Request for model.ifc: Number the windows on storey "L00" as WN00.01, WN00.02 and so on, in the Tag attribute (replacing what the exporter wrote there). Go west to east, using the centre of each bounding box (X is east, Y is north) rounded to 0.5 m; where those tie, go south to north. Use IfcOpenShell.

First a look at what the model holds.

```python
import ifcopenshell
import ifcopenshell.util.element
import ifcopenshell.util.placement

model = ifcopenshell.open("model.ifc")
print(model.schema)
storey = next(s for s in model.by_type("IfcBuildingStorey") if s.Name == "L00")
windows = [e for e in ifcopenshell.util.element.get_decomposition(storey) if e.is_a("IfcWindow")]
for e in sorted(windows, key=lambda e: e.id()):
    origin = ifcopenshell.util.placement.get_local_placement(e.ObjectPlacement)[:3, 3]
    print(e.id(), e.Tag, e.Name, origin.round(2) + 0.0, sep=" | ")
```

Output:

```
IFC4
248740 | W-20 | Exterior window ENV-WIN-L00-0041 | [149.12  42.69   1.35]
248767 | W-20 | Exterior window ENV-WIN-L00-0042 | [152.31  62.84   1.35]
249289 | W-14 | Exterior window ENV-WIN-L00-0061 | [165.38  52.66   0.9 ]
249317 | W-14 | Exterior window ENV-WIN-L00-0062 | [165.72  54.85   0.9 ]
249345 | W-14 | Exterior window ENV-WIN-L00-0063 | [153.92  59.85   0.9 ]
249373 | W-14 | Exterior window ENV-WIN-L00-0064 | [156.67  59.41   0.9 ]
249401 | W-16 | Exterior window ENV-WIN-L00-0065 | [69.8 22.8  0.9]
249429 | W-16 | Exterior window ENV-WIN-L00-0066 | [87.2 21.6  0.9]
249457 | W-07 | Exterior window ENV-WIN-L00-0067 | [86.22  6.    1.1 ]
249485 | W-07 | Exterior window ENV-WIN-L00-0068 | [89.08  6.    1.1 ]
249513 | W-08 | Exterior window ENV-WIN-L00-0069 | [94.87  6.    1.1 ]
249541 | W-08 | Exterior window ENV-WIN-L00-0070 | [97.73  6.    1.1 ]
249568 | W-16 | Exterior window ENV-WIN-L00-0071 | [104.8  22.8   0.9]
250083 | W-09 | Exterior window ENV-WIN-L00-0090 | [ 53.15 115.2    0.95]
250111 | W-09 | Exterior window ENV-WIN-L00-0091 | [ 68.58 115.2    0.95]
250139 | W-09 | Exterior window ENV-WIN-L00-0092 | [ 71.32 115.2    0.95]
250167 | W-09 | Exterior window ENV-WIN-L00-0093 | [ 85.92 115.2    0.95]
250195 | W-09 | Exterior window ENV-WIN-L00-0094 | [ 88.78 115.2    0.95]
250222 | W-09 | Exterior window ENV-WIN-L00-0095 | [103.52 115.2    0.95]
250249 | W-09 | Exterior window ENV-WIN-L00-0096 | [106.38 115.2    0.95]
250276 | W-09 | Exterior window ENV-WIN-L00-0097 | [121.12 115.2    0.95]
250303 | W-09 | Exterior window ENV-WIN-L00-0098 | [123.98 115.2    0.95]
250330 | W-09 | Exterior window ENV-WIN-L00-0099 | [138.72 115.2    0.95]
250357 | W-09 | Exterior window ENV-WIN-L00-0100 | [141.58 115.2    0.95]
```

```python
import ifcopenshell
import ifcopenshell.geom
import ifcopenshell.util.element
import ifcopenshell.util.shape

model = ifcopenshell.open("model.ifc")
settings = ifcopenshell.geom.settings()
settings.set("use-world-coords", True)


def centre(element):
    shape = ifcopenshell.geom.create_shape(settings, element)
    return ifcopenshell.util.shape.get_bbox_centroid(shape.geometry)


storey = next(s for s in model.by_type("IfcBuildingStorey") if s.Name == "L00")
windows = [e for e in ifcopenshell.util.element.get_decomposition(storey) if e.is_a("IfcWindow")]

# Insertion points can sit at a corner or the storey origin, so sort by the geometry (in metres).
centres = {e: centre(e) for e in windows}
windows.sort(key=lambda e: (round(centres[e][0] / 0.5), centres[e][1]))

for i, e in enumerate(windows, start=1):
    number = f"WN00.{i:02d}"
    e.Tag = number
    print(e.id(), number)

model.write("model_rev.ifc")
```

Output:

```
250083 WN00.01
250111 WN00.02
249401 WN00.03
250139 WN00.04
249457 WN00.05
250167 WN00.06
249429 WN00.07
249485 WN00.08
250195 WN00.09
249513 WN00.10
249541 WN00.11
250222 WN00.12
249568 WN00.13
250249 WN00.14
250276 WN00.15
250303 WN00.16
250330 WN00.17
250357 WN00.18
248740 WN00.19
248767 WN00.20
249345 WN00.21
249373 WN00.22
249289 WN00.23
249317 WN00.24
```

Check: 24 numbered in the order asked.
